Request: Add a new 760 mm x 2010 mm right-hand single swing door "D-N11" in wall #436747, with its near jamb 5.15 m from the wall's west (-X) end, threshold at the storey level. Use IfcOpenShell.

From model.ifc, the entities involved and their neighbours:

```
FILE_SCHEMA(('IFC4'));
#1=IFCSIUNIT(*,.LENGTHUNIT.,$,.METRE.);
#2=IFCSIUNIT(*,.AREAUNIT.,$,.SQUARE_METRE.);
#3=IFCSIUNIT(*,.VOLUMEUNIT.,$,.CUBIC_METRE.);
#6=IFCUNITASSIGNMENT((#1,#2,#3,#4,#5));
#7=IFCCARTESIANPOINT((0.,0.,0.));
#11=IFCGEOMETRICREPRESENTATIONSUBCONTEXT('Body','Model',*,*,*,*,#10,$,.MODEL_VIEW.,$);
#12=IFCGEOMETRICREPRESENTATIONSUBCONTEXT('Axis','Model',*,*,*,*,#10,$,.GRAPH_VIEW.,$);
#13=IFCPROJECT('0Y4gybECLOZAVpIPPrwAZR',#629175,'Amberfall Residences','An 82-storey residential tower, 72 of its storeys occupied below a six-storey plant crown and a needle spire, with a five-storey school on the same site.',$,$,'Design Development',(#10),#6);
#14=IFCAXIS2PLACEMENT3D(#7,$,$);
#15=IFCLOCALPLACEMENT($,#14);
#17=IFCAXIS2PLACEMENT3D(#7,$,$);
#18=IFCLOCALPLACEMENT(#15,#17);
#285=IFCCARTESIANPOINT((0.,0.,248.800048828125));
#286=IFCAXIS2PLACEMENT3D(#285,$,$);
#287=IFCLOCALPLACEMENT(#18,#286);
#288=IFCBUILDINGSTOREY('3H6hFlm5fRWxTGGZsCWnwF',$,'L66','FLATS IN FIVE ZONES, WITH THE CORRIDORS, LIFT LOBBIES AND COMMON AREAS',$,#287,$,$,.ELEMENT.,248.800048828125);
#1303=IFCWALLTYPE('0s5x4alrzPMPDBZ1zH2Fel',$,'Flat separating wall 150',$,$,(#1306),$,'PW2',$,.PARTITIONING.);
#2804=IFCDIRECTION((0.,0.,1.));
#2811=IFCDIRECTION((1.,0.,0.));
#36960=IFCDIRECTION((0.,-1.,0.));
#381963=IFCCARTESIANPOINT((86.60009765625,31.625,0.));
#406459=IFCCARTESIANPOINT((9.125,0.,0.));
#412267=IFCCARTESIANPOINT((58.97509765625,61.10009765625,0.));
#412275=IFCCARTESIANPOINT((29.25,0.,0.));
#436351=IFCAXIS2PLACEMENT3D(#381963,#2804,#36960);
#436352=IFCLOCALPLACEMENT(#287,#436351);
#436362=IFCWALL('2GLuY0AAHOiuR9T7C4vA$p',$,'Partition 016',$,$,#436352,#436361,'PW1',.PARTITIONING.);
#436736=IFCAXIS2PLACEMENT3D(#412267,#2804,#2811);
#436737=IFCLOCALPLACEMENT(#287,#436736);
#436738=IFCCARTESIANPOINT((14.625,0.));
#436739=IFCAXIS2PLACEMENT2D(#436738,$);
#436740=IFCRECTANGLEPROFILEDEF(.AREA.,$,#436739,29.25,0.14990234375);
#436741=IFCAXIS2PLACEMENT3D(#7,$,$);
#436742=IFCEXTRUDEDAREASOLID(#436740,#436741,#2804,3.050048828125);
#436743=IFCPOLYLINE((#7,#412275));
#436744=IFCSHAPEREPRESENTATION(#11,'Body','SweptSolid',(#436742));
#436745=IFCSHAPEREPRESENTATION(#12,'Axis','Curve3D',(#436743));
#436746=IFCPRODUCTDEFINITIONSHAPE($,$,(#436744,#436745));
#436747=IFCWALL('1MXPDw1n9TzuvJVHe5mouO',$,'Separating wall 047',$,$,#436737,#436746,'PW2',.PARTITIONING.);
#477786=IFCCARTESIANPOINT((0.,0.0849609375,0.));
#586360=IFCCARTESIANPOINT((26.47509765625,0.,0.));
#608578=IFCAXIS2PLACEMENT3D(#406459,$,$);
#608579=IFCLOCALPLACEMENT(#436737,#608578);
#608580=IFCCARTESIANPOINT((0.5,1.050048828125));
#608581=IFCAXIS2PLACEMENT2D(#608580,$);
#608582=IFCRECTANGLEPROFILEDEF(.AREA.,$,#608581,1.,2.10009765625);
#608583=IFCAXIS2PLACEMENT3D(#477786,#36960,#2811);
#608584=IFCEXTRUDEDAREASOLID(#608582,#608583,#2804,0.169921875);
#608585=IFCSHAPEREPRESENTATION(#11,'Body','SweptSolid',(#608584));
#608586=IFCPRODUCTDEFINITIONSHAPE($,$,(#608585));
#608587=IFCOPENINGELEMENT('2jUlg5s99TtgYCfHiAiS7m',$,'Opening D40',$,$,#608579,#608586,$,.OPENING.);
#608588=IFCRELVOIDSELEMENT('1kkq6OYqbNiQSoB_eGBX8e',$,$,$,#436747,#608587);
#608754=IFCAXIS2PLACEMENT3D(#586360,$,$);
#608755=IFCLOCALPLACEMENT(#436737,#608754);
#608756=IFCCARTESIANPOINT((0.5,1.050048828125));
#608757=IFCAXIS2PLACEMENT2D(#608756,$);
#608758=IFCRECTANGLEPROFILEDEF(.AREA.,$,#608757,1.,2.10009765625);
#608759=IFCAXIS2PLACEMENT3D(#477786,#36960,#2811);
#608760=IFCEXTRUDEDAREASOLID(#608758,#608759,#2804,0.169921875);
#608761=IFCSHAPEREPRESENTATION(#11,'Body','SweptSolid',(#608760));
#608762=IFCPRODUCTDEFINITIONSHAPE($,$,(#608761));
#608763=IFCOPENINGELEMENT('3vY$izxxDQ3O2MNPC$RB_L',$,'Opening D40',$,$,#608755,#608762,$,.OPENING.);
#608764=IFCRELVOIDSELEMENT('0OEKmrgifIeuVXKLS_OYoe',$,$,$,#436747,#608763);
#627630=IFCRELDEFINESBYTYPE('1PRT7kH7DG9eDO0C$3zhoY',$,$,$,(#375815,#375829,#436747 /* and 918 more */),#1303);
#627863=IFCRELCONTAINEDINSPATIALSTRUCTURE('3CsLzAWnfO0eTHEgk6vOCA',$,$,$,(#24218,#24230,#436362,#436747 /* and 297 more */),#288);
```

```python
import numpy as np
import ifcopenshell
import ifcopenshell.api.feature
import ifcopenshell.api.geometry
import ifcopenshell.api.root
import ifcopenshell.api.spatial
import ifcopenshell.geom
import ifcopenshell.util.element
import ifcopenshell.util.placement
import ifcopenshell.util.representation
import ifcopenshell.util.shape
import ifcopenshell.util.unit

model = ifcopenshell.open("model.ifc")
unit_scale = ifcopenshell.util.unit.calculate_unit_scale(model)
settings = ifcopenshell.geom.settings()


def volume(element):
    """Net volume in cubic metres, openings subtracted."""
    shape = ifcopenshell.geom.create_shape(settings, element)
    return ifcopenshell.util.shape.get_volume(shape.geometry)


wall = model.by_guid("1MXPDw1n9TzuvJVHe5mouO")
storey = ifcopenshell.util.element.get_container(wall, ifc_class="IfcBuildingStorey")
context = ifcopenshell.util.representation.get_context(model, "Model", "Body", "MODEL_VIEW")
before = volume(wall)

width, height, from_end, sill = 0.76, 2.01, 5.15, 0.0  # metres

# The wall runs along its own X axis, and the end named is its -X end.
wall_shape = ifcopenshell.geom.create_shape(settings, wall)
x, y, z = ifcopenshell.util.shape.get_vertices(wall_shape.geometry).T
start = x.min() + from_end
face, thickness = float(y.min()), float(y.max() - y.min())
wall_matrix = ifcopenshell.util.placement.get_local_placement(wall.ObjectPlacement)
level = ifcopenshell.util.placement.get_local_placement(storey.ObjectPlacement)[2, 3]


def in_wall(x, y):
    """Placement at x, y metres in the wall's axes, at sill height."""
    matrix = wall_matrix.copy()
    matrix[:, 3] = wall_matrix @ np.array([x / unit_scale, y / unit_scale, 0.0, 1.0])
    matrix[2, 3] = level + sill / unit_scale
    return matrix


# Opening: a box that overshoots both wall faces by 50 mm.
opening = ifcopenshell.api.root.create_entity(model, ifc_class="IfcOpeningElement", predefined_type="OPENING")
box = ifcopenshell.api.geometry.add_wall_representation(
    model, context=context, length=width, height=height, thickness=thickness + 0.1
)
ifcopenshell.api.geometry.assign_representation(model, product=opening, representation=box)
ifcopenshell.api.geometry.edit_object_placement(model, product=opening, matrix=in_wall(start, face - 0.05), is_si=False)
ifcopenshell.api.feature.add_feature(model, feature=opening, element=wall)

door = ifcopenshell.api.root.create_entity(model, ifc_class="IfcDoor", name="D-N11", predefined_type="DOOR")
door.OverallWidth, door.OverallHeight = width / unit_scale, height / unit_scale
door.OperationType = "SINGLE_SWING_RIGHT"
body = ifcopenshell.api.geometry.add_door_representation(
    model,
    context=context,
    overall_width=door.OverallWidth,
    overall_height=door.OverallHeight,
    operation_type="SINGLE_SWING_RIGHT",
    lining_properties={"LiningDepth": thickness / unit_scale, "ThresholdDepth": thickness / unit_scale},
)
ifcopenshell.api.geometry.assign_representation(model, product=door, representation=body)
ifcopenshell.api.spatial.assign_container(model, products=[door], relating_structure=storey)
ifcopenshell.api.feature.add_filling(model, opening=opening, element=door)

# The lining spans the wall, so the door starts at the wall face.
ifcopenshell.api.geometry.edit_object_placement(model, product=door, matrix=in_wall(start, face), is_si=False)

after = volume(wall)

print(f"wall volume {before:.3f} -> {after:.3f} m3")

model.write("model_v2.ifc")
```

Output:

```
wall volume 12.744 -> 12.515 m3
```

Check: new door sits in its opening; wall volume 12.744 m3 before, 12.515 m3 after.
